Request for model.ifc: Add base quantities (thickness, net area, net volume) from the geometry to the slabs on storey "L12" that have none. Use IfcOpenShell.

First a look at what the model holds.

```python
import ifcopenshell
import ifcopenshell.util.element
import ifcopenshell.util.unit

model = ifcopenshell.open("model.ifc")
print(model.schema)
for unit_type in ("LENGTHUNIT", "AREAUNIT", "VOLUMEUNIT"):
    print(unit_type, ifcopenshell.util.unit.calculate_unit_scale(model, unit_type))
storey = next(s for s in model.by_type("IfcBuildingStorey") if s.Name == "L12")
slabs = [e for e in ifcopenshell.util.element.get_decomposition(storey) if e.is_a("IfcSlab")]
for e in sorted(slabs, key=lambda e: e.id()):
    print(e.id(), e.is_a(), e.Name, list(ifcopenshell.util.element.get_psets(e, qtos_only=True)), sep=" | ")
```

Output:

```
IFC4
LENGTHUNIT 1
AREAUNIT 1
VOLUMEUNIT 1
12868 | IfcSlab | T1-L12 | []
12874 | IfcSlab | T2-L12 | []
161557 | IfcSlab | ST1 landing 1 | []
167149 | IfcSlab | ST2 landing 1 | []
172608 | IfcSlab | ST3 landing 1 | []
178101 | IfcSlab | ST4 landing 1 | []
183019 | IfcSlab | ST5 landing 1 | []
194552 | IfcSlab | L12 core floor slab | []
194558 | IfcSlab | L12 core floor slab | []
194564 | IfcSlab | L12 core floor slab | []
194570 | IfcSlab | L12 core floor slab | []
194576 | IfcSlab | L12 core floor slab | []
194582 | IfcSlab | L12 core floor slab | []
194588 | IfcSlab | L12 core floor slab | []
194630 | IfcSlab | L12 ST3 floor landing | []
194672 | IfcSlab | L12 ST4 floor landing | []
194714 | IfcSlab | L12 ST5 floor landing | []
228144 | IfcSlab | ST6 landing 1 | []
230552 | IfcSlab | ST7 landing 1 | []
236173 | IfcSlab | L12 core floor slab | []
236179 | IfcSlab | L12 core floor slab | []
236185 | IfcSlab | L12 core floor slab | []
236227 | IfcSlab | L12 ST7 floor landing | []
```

```python
import ifcopenshell
import ifcopenshell.api.pset
import ifcopenshell.geom
import ifcopenshell.util.element
import ifcopenshell.util.shape
import ifcopenshell.util.unit

model = ifcopenshell.open("model.ifc")
unit_scale = ifcopenshell.util.unit.calculate_unit_scale(model)
area_scale = ifcopenshell.util.unit.calculate_unit_scale(model, "AREAUNIT")
volume_scale = ifcopenshell.util.unit.calculate_unit_scale(model, "VOLUMEUNIT")
settings = ifcopenshell.geom.settings()

storey = next(s for s in model.by_type("IfcBuildingStorey") if s.Name == "L12")
slabs = [e for e in ifcopenshell.util.element.get_decomposition(storey) if e.is_a("IfcSlab")]

for e in sorted(slabs, key=lambda e: e.id()):
    if ifcopenshell.util.element.get_psets(e, qtos_only=True, should_inherit=False):
        continue
    # Geometry comes back in metres, in the element's own axes.
    shape = ifcopenshell.geom.create_shape(settings, e)
    values = {
        "Width": ifcopenshell.util.shape.get_z(shape.geometry) / unit_scale,
        "NetArea": ifcopenshell.util.shape.get_footprint_area(shape.geometry) / area_scale,
        "NetVolume": ifcopenshell.util.shape.get_volume(shape.geometry) / volume_scale,
    }
    qto = ifcopenshell.api.pset.add_qto(model, product=e, name="Qto_SlabBaseQuantities")
    ifcopenshell.api.pset.edit_qto(model, qto=qto, properties=values)
    print(e.id(), {k: round(v, 3) for k, v in values.items()})

model.write("model_v2.ifc")
```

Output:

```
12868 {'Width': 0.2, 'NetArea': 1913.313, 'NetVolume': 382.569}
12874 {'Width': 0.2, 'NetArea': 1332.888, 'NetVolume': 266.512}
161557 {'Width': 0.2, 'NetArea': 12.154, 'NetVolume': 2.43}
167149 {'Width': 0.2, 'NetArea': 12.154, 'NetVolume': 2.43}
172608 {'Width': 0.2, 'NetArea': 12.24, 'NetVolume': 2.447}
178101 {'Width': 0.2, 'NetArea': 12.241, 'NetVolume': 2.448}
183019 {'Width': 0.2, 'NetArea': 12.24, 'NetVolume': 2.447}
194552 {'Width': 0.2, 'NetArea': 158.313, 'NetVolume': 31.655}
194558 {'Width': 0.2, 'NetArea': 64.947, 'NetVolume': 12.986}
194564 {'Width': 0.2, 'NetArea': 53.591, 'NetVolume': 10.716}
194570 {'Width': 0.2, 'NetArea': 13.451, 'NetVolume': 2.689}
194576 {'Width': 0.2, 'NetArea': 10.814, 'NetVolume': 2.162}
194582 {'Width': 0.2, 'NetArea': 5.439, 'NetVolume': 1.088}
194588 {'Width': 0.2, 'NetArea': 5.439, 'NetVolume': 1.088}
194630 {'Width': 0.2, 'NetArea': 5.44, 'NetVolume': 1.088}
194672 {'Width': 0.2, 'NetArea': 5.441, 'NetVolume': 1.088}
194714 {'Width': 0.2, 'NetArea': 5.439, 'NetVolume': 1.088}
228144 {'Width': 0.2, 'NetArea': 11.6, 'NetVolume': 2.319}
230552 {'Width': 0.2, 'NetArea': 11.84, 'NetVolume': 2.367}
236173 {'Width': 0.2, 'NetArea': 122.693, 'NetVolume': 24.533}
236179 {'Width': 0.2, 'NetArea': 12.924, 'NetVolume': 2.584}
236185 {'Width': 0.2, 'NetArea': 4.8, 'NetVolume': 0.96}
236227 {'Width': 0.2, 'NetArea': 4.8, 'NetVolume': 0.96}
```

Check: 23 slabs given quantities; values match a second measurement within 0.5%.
